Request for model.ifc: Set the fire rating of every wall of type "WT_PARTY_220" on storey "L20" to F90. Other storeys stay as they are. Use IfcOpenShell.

First a look at what the model holds.

```python
import ifcopenshell
import ifcopenshell.util.element

model = ifcopenshell.open("model.ifc")
print(model.schema)
storey = next(s for s in model.by_type("IfcBuildingStorey") if s.Name == "L20")
walls = [e for e in ifcopenshell.util.element.get_decomposition(storey) if e.is_a("IfcWall")]
seen = {}
for e in walls:
    element_type = ifcopenshell.util.element.get_type(e)
    key = (element_type.Name if element_type != e and element_type else None, ifcopenshell.util.element.get_pset(e, "Pset_WallCommon", "FireRating"))
    seen[key] = seen.get(key, 0) + 1
for (name, value), count in sorted(seen.items(), key=str):
    print(count, "x", name, "|", value)
```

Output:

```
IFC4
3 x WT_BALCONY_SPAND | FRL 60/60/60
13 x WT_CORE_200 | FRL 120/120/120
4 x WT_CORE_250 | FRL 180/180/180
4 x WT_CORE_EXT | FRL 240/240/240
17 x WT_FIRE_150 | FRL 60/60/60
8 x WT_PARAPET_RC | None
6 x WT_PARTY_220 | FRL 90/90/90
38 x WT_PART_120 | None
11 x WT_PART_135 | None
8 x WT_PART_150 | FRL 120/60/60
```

```python
import ifcopenshell
import ifcopenshell.api.pset
import ifcopenshell.util.element

model = ifcopenshell.open("model.ifc")

storey = next(s for s in model.by_type("IfcBuildingStorey") if s.Name == "L20")
walls = [e for e in ifcopenshell.util.element.get_decomposition(storey) if e.is_a("IfcWall")]

count = 0
for e in walls:
    element_type = ifcopenshell.util.element.get_type(e)
    if element_type in (None, e) or element_type.Name != "WT_PARTY_220":
        continue
    # add_pset returns the element's existing set when there is one.
    pset = ifcopenshell.api.pset.add_pset(model, product=e, name="Pset_WallCommon")
    ifcopenshell.api.pset.edit_pset(model, pset=pset, properties={"FireRating": "F90"})
    count += 1

print(count, "walls updated")

model.write("model-out.ifc")
```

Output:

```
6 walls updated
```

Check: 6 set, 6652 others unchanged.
